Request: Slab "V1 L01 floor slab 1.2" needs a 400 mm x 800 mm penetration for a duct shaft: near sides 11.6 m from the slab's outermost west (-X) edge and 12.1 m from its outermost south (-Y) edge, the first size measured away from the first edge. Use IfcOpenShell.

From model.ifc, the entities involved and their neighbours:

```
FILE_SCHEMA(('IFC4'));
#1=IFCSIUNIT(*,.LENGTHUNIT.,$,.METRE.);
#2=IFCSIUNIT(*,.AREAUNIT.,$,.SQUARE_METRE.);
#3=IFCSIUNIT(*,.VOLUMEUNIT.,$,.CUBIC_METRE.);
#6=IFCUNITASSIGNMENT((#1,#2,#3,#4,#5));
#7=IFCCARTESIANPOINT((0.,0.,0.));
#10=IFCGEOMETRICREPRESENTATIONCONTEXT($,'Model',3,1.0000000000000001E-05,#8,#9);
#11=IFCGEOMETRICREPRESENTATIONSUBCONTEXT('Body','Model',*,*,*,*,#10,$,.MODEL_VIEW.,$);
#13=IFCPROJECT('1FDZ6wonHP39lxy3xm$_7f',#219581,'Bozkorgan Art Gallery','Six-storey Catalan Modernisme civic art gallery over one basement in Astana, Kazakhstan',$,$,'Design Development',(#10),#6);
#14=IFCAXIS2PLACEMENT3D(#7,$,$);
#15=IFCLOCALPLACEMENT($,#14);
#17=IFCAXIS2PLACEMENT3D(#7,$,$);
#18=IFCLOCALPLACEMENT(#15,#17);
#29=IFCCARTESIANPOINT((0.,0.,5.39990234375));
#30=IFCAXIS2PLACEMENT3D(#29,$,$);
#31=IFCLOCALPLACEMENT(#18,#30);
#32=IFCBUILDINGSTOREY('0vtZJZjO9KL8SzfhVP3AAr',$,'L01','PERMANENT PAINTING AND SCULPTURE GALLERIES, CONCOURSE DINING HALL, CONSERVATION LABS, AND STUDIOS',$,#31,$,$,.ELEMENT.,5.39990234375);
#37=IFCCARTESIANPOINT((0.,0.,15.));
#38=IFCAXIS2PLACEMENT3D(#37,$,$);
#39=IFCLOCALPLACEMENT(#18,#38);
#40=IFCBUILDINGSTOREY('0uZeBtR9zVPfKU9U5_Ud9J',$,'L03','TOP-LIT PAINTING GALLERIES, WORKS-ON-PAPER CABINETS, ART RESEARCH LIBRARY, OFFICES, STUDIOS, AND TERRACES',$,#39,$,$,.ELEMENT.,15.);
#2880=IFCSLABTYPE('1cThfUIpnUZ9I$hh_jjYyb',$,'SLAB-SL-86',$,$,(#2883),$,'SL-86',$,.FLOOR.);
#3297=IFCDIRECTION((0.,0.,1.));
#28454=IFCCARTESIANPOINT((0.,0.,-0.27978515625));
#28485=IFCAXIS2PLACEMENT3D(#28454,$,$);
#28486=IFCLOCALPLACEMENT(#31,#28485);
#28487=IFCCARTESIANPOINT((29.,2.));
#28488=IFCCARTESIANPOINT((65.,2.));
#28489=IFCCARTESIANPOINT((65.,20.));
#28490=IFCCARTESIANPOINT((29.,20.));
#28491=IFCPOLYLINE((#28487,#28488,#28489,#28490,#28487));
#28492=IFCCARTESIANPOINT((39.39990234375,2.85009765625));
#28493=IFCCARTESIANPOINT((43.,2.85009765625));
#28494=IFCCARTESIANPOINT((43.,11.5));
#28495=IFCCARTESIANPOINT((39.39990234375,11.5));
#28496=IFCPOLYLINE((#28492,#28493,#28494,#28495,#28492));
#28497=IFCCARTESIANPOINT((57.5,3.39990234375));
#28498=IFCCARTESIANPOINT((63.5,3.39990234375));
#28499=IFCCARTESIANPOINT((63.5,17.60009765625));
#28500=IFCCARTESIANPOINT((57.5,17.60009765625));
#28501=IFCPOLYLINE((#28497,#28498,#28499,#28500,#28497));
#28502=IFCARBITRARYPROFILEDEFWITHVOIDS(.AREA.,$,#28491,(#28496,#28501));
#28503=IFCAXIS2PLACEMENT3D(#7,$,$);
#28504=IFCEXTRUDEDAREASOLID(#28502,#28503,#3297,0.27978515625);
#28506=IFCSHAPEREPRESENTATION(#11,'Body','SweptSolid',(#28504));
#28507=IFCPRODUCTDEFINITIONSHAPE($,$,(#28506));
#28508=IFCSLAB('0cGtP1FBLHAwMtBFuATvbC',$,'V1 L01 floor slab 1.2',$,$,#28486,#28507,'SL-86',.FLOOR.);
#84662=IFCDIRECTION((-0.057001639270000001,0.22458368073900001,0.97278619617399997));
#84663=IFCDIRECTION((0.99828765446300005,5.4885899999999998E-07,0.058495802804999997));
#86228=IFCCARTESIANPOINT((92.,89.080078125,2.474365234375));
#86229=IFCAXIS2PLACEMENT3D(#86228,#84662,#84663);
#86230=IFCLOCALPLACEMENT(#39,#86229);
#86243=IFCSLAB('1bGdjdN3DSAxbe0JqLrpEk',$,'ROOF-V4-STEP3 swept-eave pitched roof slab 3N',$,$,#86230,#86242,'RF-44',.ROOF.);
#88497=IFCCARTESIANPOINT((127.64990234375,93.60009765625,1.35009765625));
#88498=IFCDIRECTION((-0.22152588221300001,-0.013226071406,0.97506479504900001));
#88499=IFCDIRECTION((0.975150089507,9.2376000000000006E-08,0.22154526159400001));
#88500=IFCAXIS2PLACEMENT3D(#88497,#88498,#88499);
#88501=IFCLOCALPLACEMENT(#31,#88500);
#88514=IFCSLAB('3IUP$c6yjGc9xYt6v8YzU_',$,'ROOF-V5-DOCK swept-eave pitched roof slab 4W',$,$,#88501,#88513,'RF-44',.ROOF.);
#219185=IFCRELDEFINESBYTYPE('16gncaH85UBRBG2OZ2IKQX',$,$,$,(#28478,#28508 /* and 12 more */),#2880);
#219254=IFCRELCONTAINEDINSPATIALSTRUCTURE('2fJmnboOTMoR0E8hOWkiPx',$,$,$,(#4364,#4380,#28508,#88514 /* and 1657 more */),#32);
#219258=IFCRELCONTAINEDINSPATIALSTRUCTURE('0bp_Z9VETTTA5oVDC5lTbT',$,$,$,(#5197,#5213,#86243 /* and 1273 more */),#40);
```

```python
import numpy as np
import ifcopenshell
import ifcopenshell.api.feature
import ifcopenshell.api.geometry
import ifcopenshell.api.root
import ifcopenshell.geom
import ifcopenshell.util.placement
import ifcopenshell.util.representation
import ifcopenshell.util.shape
import ifcopenshell.util.unit

model = ifcopenshell.open("model.ifc")
unit_scale = ifcopenshell.util.unit.calculate_unit_scale(model)
settings = ifcopenshell.geom.settings()


def volume(element):
    """Net volume in cubic metres, openings subtracted."""
    shape = ifcopenshell.geom.create_shape(settings, element)
    return ifcopenshell.util.shape.get_volume(shape.geometry)


slab = model.by_guid("0cGtP1FBLHAwMtBFuATvbC")
before = volume(slab)

# Extent in the slab's own axes, in metres. The edges named are its -X and -Y sides.
slab_shape = ifcopenshell.geom.create_shape(settings, slab)
vertices = ifcopenshell.util.shape.get_vertices(slab_shape.geometry)
x_min, y_min, bottom = vertices.min(axis=0)
top = vertices[:, 2].max()

opening = ifcopenshell.api.root.create_entity(model, ifc_class="IfcOpeningElement", name="Duct shaft opening", predefined_type="OPENING")
context = ifcopenshell.util.representation.get_context(model, "Model", "Body", "MODEL_VIEW")
width, depth = 0.4, 0.8
outline = [(0.0, 0.0), (width, 0.0), (width, depth), (0.0, depth), (0.0, 0.0)]
# Overshoot both faces by 50 mm so the cut is clean.
shape = ifcopenshell.api.geometry.add_slab_representation(
    model, context=context, depth=top - bottom + 0.1, polyline=outline
)
ifcopenshell.api.geometry.assign_representation(model, product=opening, representation=shape)

matrix = ifcopenshell.util.placement.get_local_placement(slab.ObjectPlacement)
matrix[:, 3] = matrix @ np.append(np.array([x_min + 11.6, y_min + 12.1, bottom - 0.05]) / unit_scale, 1.0)
ifcopenshell.api.geometry.edit_object_placement(model, product=opening, matrix=matrix, is_si=False)
ifcopenshell.api.feature.add_feature(model, feature=opening, element=slab)

after = volume(slab)

print(f"slab volume {before:.3f} -> {after:.3f} m3")

model.write("model-out.ifc")
```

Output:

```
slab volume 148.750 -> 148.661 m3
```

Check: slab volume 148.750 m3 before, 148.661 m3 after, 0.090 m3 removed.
